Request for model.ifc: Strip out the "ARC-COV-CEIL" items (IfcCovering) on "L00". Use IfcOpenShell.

First a look at what the model holds.

```python
import ifcopenshell
import ifcopenshell.util.element

model = ifcopenshell.open("model.ifc")
print(model.schema)
storey = next(s for s in model.by_type("IfcBuildingStorey") if s.Name == "L00")
coverings = [e for e in ifcopenshell.util.element.get_decomposition(storey) if e.is_a("IfcCovering")]
seen = {}
for e in coverings:
    element_type = ifcopenshell.util.element.get_type(e)
    name = element_type.Name if element_type not in (None, e) else None
    seen[name] = seen.get(name, 0) + 1
for name, count in sorted(seen.items(), key=str):
    print(count, "x", name)
```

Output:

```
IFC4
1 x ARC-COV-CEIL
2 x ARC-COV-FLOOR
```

```python
import ifcopenshell
import ifcopenshell.api.root
import ifcopenshell.util.element

model = ifcopenshell.open("model.ifc")

storey = next(s for s in model.by_type("IfcBuildingStorey") if s.Name == "L00")
coverings = [e for e in ifcopenshell.util.element.get_decomposition(storey) if e.is_a("IfcCovering")]
targets = [e for e in coverings if (t := ifcopenshell.util.element.get_type(e)) not in (None, e) and t.Name == "ARC-COV-CEIL"]

for e in targets:
    ifcopenshell.api.root.remove_product(model, product=e)
print(len(targets), "removed")

model.write("model_v2.ifc")
```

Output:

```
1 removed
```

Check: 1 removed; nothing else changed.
